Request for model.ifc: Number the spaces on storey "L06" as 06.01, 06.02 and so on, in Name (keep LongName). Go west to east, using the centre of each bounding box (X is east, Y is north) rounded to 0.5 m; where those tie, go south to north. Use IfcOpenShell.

First a look at what the model holds.

```python
import ifcopenshell
import ifcopenshell.util.element
import ifcopenshell.util.placement

model = ifcopenshell.open("model.ifc")
print(model.schema)
storey = next(s for s in model.by_type("IfcBuildingStorey") if s.Name == "L06")
spaces = [e for e in ifcopenshell.util.element.get_decomposition(storey) if e.is_a("IfcSpace")]
for e in sorted(spaces, key=lambda e: e.id()):
    origin = ifcopenshell.util.placement.get_local_placement(e.ObjectPlacement)[:3, 3]
    print(e.id(), e.Name, e.LongName, origin.round(2) + 0.0, sep=" | ")
```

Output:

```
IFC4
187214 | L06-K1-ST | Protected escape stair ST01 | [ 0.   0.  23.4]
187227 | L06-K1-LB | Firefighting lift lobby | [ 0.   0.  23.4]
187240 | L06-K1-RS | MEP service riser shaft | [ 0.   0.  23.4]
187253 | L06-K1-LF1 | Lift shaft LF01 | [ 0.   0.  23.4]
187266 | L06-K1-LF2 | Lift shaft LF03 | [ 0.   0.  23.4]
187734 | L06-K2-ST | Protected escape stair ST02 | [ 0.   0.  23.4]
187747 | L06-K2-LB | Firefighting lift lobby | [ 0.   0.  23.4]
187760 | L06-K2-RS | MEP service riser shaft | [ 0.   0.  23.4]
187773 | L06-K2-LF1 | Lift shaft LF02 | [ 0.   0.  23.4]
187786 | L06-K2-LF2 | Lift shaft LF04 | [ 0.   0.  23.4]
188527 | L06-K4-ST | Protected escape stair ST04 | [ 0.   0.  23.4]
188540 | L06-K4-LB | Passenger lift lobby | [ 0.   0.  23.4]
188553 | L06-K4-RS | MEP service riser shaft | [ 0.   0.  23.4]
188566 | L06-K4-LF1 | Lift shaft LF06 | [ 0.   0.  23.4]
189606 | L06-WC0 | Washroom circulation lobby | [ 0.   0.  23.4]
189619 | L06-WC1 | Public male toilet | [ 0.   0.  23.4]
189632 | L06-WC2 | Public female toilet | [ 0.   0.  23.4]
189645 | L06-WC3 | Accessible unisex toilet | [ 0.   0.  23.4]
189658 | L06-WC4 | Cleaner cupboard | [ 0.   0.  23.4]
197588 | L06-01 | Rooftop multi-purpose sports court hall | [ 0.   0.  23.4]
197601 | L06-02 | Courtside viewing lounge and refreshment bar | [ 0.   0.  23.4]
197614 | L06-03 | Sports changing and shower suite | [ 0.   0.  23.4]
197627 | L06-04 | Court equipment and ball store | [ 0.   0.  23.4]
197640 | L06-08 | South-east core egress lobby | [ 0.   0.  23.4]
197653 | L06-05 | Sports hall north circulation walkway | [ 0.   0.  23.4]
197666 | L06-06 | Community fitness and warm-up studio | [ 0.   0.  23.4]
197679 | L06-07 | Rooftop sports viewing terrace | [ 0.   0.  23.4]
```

```python
import ifcopenshell
import ifcopenshell.geom
import ifcopenshell.util.element
import ifcopenshell.util.shape

model = ifcopenshell.open("model.ifc")
settings = ifcopenshell.geom.settings()
settings.set("use-world-coords", True)


def centre(element):
    shape = ifcopenshell.geom.create_shape(settings, element)
    return ifcopenshell.util.shape.get_bbox_centroid(shape.geometry)


storey = next(s for s in model.by_type("IfcBuildingStorey") if s.Name == "L06")
spaces = [e for e in ifcopenshell.util.element.get_decomposition(storey) if e.is_a("IfcSpace")]

# Insertion points can sit at a corner or the storey origin, so sort by the geometry (in metres).
centres = {e: centre(e) for e in spaces}
spaces.sort(key=lambda e: (round(centres[e][0] / 0.5), centres[e][1]))

for i, e in enumerate(spaces, start=1):
    number = f"06.{i:02d}"
    e.Name = number
    print(e.id(), number)

model.write("model_v2.ifc")
```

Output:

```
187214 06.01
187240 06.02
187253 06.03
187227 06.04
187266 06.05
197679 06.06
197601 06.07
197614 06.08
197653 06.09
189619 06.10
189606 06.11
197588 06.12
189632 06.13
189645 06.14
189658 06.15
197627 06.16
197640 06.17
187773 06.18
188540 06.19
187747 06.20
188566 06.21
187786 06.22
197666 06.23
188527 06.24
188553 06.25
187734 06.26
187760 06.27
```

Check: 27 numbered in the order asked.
